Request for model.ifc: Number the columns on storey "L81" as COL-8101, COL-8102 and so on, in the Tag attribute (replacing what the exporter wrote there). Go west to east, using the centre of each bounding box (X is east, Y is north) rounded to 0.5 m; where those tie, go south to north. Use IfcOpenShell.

First a look at what the model holds.

```python
import ifcopenshell
import ifcopenshell.util.element
import ifcopenshell.util.placement

model = ifcopenshell.open("model.ifc")
print(model.schema)
storey = next(s for s in model.by_type("IfcBuildingStorey") if s.Name == "L81")
columns = [e for e in ifcopenshell.util.element.get_decomposition(storey) if e.is_a("IfcColumn")]
for e in sorted(columns, key=lambda e: e.id()):
    origin = ifcopenshell.util.placement.get_local_placement(e.ObjectPlacement)[:3, 3]
    print(e.id(), e.Tag, e.Name, origin.round(2) + 0.0, sep=" | ")
```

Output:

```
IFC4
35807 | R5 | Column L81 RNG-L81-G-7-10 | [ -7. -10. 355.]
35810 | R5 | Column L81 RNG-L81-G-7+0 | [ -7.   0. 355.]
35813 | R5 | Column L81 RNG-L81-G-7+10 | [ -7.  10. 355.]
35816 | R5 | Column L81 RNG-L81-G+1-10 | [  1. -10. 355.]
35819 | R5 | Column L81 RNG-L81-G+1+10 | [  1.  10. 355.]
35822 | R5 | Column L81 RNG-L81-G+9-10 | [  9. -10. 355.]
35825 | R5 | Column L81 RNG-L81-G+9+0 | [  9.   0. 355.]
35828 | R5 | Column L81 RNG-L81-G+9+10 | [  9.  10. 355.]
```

```python
import ifcopenshell
import ifcopenshell.geom
import ifcopenshell.util.element
import ifcopenshell.util.shape

model = ifcopenshell.open("model.ifc")
settings = ifcopenshell.geom.settings()
settings.set("use-world-coords", True)


def centre(element):
    shape = ifcopenshell.geom.create_shape(settings, element)
    return ifcopenshell.util.shape.get_bbox_centroid(shape.geometry)


storey = next(s for s in model.by_type("IfcBuildingStorey") if s.Name == "L81")
columns = [e for e in ifcopenshell.util.element.get_decomposition(storey) if e.is_a("IfcColumn")]

# Insertion points can sit at a corner or the storey origin, so sort by the geometry (in metres).
centres = {e: centre(e) for e in columns}
columns.sort(key=lambda e: (round(centres[e][0] / 0.5), centres[e][1]))

for i, e in enumerate(columns, start=1):
    number = f"COL-81{i:02d}"
    e.Tag = number
    print(e.id(), number)

model.write("model_edited.ifc")
```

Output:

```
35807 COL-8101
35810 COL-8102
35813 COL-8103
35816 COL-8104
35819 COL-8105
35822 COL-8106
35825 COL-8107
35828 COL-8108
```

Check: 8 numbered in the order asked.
